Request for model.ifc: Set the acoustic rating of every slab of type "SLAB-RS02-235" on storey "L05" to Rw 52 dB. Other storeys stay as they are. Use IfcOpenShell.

First a look at what the model holds.

```python
import ifcopenshell
import ifcopenshell.util.element

model = ifcopenshell.open("model.ifc")
print(model.schema)
storey = next(s for s in model.by_type("IfcBuildingStorey") if s.Name == "L05")
slabs = [e for e in ifcopenshell.util.element.get_decomposition(storey) if e.is_a("IfcSlab")]
seen = {}
for e in slabs:
    element_type = ifcopenshell.util.element.get_type(e)
    key = (element_type.Name if element_type != e and element_type else None, ifcopenshell.util.element.get_pset(e, "Pset_SlabCommon", "AcousticRating"))
    seen[key] = seen.get(key, 0) + 1
for (name, value), count in sorted(seen.items(), key=str):
    print(count, "x", name, "|", value)
```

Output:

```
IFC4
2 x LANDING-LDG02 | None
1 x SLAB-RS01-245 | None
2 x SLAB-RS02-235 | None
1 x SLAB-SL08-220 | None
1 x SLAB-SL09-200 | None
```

```python
import ifcopenshell
import ifcopenshell.api.pset
import ifcopenshell.util.element

model = ifcopenshell.open("model.ifc")

storey = next(s for s in model.by_type("IfcBuildingStorey") if s.Name == "L05")
slabs = [e for e in ifcopenshell.util.element.get_decomposition(storey) if e.is_a("IfcSlab")]

count = 0
for e in slabs:
    element_type = ifcopenshell.util.element.get_type(e)
    if element_type in (None, e) or element_type.Name != "SLAB-RS02-235":
        continue
    # add_pset returns the element's existing set when there is one.
    pset = ifcopenshell.api.pset.add_pset(model, product=e, name="Pset_SlabCommon")
    ifcopenshell.api.pset.edit_pset(model, pset=pset, properties={"AcousticRating": "Rw 52 dB"})
    count += 1

print(count, "slabs updated")

model.write("model_rev.ifc")
```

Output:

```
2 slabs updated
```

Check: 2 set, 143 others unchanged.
